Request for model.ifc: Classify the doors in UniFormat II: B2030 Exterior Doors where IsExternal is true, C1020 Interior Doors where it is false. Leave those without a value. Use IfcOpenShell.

First a look at what the model holds.

```python
import ifcopenshell
import ifcopenshell.util.element

model = ifcopenshell.open("model.ifc")
print(model.schema)
print("classifications:", [c.Name for c in model.by_type("IfcClassification")])
values = [ifcopenshell.util.element.get_pset(e, "Pset_DoorCommon", "IsExternal") for e in model.by_type("IfcDoor")]
for value in (True, False, None):
    print("IsExternal", value, values.count(value))
```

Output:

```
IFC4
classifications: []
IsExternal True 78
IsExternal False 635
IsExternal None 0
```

```python
import ifcopenshell
import ifcopenshell.api.classification
import ifcopenshell.util.element

model = ifcopenshell.open("model.ifc")

system = ifcopenshell.api.classification.add_classification(model, classification="UniFormat II")

doors = model.by_type("IfcDoor")
external = {e: ifcopenshell.util.element.get_pset(e, "Pset_DoorCommon", "IsExternal") for e in doors}
for flag, code, name in ((True, "B2030", "Exterior Doors"), (False, "C1020", "Interior Doors")):
    products = [e for e in doors if external[e] is flag]
    ifcopenshell.api.classification.add_reference(
        model, products=products, classification=system, identification=code, name=name
    )
    print(code, len(products))

model.write("model_updated.ifc")
```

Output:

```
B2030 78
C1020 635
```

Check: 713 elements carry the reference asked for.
